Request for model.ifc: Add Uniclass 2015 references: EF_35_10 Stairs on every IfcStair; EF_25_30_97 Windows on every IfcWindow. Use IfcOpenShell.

First a look at what the model holds.

```python
import ifcopenshell

model = ifcopenshell.open("model.ifc")
print(model.schema)
print("classifications:", [c.Name for c in model.by_type("IfcClassification")])
for ifc_class in ("IfcDoor", "IfcRoof", "IfcStair", "IfcWall", "IfcWindow"):
    print(ifc_class, len(model.by_type(ifc_class)))
```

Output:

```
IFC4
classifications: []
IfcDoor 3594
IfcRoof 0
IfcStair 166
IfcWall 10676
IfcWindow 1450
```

```python
import ifcopenshell
import ifcopenshell.api.classification

model = ifcopenshell.open("model.ifc")

system = ifcopenshell.api.classification.add_classification(model, classification="Uniclass 2015")

codes = {
    "IfcStair": ("EF_35_10", "Stairs"),
    "IfcWindow": ("EF_25_30_97", "Windows"),
}
for ifc_class, (code, name) in codes.items():
    products = model.by_type(ifc_class)
    ifcopenshell.api.classification.add_reference(
        model, products=products, classification=system, identification=code, name=name
    )
    print(code, len(products))

model.write("model_updated.ifc")
```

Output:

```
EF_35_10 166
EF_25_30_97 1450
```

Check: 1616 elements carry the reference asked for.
